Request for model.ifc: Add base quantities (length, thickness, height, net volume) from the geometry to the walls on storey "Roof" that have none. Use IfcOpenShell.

First a look at what the model holds.

```python
import ifcopenshell
import ifcopenshell.util.element
import ifcopenshell.util.unit

model = ifcopenshell.open("model.ifc")
print(model.schema)
for unit_type in ("LENGTHUNIT", "AREAUNIT", "VOLUMEUNIT"):
    print(unit_type, ifcopenshell.util.unit.calculate_unit_scale(model, unit_type))
storey = next(s for s in model.by_type("IfcBuildingStorey") if s.Name == "Roof")
walls = [e for e in ifcopenshell.util.element.get_decomposition(storey) if e.is_a("IfcWall")]
for e in sorted(walls, key=lambda e: e.id()):
    print(e.id(), e.is_a(), e.Name, list(ifcopenshell.util.element.get_psets(e, qtos_only=True)), sep=" | ")
```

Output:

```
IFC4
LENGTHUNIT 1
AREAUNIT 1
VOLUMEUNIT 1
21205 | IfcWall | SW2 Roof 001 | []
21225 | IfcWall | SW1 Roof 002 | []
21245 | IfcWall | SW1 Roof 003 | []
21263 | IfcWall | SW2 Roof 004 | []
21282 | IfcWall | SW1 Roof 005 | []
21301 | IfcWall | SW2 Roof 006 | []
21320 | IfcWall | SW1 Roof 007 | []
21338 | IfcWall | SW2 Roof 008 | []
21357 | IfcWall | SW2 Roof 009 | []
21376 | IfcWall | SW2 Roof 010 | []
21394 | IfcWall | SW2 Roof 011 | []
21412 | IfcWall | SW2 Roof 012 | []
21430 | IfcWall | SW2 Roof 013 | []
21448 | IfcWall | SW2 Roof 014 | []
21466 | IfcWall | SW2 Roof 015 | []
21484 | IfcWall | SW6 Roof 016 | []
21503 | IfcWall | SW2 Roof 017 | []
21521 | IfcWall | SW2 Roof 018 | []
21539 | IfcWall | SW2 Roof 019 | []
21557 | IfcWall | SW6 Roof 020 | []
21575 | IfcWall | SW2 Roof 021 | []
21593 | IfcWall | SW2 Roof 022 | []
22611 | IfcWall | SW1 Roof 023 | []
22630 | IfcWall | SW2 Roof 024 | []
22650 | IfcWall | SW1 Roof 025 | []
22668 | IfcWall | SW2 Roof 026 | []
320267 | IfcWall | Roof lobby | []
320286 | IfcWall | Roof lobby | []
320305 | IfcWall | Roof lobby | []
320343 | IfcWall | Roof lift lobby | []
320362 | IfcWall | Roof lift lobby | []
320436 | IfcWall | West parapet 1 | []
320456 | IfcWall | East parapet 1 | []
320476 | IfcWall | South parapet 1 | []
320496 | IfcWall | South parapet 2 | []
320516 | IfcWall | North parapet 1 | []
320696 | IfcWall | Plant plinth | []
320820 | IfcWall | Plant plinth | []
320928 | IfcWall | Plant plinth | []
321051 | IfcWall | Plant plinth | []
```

```python
import ifcopenshell
import ifcopenshell.api.pset
import ifcopenshell.geom
import ifcopenshell.util.element
import ifcopenshell.util.shape
import ifcopenshell.util.unit

model = ifcopenshell.open("model.ifc")
unit_scale = ifcopenshell.util.unit.calculate_unit_scale(model)
volume_scale = ifcopenshell.util.unit.calculate_unit_scale(model, "VOLUMEUNIT")
settings = ifcopenshell.geom.settings()

storey = next(s for s in model.by_type("IfcBuildingStorey") if s.Name == "Roof")
walls = [e for e in ifcopenshell.util.element.get_decomposition(storey) if e.is_a("IfcWall")]

for e in sorted(walls, key=lambda e: e.id()):
    if ifcopenshell.util.element.get_psets(e, qtos_only=True, should_inherit=False):
        continue
    # Geometry comes back in metres, in the element's own axes.
    shape = ifcopenshell.geom.create_shape(settings, e)
    values = {
        "Length": ifcopenshell.util.shape.get_x(shape.geometry) / unit_scale,
        "Width": ifcopenshell.util.shape.get_y(shape.geometry) / unit_scale,
        "Height": ifcopenshell.util.shape.get_z(shape.geometry) / unit_scale,
        "NetVolume": ifcopenshell.util.shape.get_volume(shape.geometry) / volume_scale,
    }
    qto = ifcopenshell.api.pset.add_qto(model, product=e, name="Qto_WallBaseQuantities")
    ifcopenshell.api.pset.edit_qto(model, qto=qto, properties=values)
    print(e.id(), {k: round(v, 3) for k, v in values.items()})

model.write("model_rev.ifc")
```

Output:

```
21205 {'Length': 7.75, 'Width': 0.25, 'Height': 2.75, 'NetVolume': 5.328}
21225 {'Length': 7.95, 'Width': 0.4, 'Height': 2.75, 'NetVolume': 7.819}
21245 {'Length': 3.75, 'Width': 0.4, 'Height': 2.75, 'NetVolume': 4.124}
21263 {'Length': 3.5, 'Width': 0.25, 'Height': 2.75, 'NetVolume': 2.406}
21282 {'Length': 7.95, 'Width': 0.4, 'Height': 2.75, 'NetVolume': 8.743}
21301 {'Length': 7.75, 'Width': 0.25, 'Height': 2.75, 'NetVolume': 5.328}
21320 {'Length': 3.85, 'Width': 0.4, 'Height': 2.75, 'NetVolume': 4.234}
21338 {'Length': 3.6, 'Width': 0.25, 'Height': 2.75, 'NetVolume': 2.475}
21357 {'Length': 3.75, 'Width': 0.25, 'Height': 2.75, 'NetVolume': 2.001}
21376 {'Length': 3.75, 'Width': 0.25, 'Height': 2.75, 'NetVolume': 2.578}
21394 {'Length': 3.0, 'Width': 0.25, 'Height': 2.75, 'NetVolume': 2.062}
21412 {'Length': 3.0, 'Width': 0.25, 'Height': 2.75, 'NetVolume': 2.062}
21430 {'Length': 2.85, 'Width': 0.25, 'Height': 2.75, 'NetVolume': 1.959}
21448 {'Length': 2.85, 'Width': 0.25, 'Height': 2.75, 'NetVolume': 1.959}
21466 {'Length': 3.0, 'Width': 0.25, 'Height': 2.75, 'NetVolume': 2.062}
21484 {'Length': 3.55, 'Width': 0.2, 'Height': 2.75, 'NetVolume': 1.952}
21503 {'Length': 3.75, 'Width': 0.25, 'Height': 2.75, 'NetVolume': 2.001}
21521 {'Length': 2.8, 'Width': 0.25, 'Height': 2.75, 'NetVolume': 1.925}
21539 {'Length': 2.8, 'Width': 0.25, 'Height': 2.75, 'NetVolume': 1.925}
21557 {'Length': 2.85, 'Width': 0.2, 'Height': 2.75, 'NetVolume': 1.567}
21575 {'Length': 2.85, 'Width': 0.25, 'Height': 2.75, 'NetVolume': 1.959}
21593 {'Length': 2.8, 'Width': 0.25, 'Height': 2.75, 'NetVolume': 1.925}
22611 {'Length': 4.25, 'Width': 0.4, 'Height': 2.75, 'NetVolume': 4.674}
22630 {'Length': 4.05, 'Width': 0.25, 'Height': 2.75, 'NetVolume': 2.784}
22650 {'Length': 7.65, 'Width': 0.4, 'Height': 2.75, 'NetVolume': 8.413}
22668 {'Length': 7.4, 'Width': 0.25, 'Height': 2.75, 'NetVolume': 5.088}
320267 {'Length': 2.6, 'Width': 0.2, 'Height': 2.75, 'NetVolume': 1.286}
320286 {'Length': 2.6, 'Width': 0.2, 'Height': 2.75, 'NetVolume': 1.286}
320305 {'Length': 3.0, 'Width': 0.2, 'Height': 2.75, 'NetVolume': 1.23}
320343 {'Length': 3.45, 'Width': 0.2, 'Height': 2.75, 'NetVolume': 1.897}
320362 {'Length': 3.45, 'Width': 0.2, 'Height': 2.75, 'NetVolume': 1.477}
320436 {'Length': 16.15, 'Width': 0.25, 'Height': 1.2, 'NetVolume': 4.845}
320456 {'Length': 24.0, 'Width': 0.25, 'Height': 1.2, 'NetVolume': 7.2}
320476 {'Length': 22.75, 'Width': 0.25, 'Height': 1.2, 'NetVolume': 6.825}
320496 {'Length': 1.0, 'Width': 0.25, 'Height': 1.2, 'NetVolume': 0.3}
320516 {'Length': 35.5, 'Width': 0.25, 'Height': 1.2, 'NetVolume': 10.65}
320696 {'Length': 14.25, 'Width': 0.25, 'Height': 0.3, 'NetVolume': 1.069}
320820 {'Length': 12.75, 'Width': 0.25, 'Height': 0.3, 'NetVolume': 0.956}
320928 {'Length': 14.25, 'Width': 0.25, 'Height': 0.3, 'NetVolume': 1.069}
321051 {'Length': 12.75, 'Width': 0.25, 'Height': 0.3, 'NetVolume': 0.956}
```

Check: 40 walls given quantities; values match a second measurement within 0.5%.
